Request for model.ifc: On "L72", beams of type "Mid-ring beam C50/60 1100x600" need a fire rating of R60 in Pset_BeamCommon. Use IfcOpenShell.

First a look at what the model holds.

```python
import ifcopenshell
import ifcopenshell.util.element

model = ifcopenshell.open("model.ifc")
print(model.schema)
storey = next(s for s in model.by_type("IfcBuildingStorey") if s.Name == "L72")
beams = [e for e in ifcopenshell.util.element.get_decomposition(storey) if e.is_a("IfcBeam")]
seen = {}
for e in beams:
    element_type = ifcopenshell.util.element.get_type(e)
    key = (element_type.Name if element_type != e and element_type else None, ifcopenshell.util.element.get_pset(e, "Pset_BeamCommon", "FireRating"))
    seen[key] = seen.get(key, 0) + 1
for (name, value), count in sorted(seen.items(), key=str):
    print(count, "x", name, "|", value)
```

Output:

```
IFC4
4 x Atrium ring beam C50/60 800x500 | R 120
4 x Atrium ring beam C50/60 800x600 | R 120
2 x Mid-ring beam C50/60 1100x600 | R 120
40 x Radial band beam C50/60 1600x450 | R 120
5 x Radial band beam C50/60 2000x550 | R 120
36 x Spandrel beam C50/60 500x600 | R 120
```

```python
import ifcopenshell
import ifcopenshell.api.pset
import ifcopenshell.util.element

model = ifcopenshell.open("model.ifc")

storey = next(s for s in model.by_type("IfcBuildingStorey") if s.Name == "L72")
beams = [e for e in ifcopenshell.util.element.get_decomposition(storey) if e.is_a("IfcBeam")]

count = 0
for e in beams:
    element_type = ifcopenshell.util.element.get_type(e)
    if element_type in (None, e) or element_type.Name != "Mid-ring beam C50/60 1100x600":
        continue
    found = ifcopenshell.util.element.get_pset(e, "Pset_BeamCommon", should_inherit=False)
    if found:
        pset = model.by_id(found["id"])
        if len(ifcopenshell.util.element.get_elements_by_pset(pset)) > 1:
            pset = ifcopenshell.api.pset.unshare_pset(model, products=[e], pset=pset)[0]
    else:
        pset = ifcopenshell.api.pset.add_pset(model, product=e, name="Pset_BeamCommon")
    ifcopenshell.api.pset.edit_pset(model, pset=pset, properties={"FireRating": "R60"})
    count += 1

print(count, "beams updated")

model.write("model_v2.ifc")
```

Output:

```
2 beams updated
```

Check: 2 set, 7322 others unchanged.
